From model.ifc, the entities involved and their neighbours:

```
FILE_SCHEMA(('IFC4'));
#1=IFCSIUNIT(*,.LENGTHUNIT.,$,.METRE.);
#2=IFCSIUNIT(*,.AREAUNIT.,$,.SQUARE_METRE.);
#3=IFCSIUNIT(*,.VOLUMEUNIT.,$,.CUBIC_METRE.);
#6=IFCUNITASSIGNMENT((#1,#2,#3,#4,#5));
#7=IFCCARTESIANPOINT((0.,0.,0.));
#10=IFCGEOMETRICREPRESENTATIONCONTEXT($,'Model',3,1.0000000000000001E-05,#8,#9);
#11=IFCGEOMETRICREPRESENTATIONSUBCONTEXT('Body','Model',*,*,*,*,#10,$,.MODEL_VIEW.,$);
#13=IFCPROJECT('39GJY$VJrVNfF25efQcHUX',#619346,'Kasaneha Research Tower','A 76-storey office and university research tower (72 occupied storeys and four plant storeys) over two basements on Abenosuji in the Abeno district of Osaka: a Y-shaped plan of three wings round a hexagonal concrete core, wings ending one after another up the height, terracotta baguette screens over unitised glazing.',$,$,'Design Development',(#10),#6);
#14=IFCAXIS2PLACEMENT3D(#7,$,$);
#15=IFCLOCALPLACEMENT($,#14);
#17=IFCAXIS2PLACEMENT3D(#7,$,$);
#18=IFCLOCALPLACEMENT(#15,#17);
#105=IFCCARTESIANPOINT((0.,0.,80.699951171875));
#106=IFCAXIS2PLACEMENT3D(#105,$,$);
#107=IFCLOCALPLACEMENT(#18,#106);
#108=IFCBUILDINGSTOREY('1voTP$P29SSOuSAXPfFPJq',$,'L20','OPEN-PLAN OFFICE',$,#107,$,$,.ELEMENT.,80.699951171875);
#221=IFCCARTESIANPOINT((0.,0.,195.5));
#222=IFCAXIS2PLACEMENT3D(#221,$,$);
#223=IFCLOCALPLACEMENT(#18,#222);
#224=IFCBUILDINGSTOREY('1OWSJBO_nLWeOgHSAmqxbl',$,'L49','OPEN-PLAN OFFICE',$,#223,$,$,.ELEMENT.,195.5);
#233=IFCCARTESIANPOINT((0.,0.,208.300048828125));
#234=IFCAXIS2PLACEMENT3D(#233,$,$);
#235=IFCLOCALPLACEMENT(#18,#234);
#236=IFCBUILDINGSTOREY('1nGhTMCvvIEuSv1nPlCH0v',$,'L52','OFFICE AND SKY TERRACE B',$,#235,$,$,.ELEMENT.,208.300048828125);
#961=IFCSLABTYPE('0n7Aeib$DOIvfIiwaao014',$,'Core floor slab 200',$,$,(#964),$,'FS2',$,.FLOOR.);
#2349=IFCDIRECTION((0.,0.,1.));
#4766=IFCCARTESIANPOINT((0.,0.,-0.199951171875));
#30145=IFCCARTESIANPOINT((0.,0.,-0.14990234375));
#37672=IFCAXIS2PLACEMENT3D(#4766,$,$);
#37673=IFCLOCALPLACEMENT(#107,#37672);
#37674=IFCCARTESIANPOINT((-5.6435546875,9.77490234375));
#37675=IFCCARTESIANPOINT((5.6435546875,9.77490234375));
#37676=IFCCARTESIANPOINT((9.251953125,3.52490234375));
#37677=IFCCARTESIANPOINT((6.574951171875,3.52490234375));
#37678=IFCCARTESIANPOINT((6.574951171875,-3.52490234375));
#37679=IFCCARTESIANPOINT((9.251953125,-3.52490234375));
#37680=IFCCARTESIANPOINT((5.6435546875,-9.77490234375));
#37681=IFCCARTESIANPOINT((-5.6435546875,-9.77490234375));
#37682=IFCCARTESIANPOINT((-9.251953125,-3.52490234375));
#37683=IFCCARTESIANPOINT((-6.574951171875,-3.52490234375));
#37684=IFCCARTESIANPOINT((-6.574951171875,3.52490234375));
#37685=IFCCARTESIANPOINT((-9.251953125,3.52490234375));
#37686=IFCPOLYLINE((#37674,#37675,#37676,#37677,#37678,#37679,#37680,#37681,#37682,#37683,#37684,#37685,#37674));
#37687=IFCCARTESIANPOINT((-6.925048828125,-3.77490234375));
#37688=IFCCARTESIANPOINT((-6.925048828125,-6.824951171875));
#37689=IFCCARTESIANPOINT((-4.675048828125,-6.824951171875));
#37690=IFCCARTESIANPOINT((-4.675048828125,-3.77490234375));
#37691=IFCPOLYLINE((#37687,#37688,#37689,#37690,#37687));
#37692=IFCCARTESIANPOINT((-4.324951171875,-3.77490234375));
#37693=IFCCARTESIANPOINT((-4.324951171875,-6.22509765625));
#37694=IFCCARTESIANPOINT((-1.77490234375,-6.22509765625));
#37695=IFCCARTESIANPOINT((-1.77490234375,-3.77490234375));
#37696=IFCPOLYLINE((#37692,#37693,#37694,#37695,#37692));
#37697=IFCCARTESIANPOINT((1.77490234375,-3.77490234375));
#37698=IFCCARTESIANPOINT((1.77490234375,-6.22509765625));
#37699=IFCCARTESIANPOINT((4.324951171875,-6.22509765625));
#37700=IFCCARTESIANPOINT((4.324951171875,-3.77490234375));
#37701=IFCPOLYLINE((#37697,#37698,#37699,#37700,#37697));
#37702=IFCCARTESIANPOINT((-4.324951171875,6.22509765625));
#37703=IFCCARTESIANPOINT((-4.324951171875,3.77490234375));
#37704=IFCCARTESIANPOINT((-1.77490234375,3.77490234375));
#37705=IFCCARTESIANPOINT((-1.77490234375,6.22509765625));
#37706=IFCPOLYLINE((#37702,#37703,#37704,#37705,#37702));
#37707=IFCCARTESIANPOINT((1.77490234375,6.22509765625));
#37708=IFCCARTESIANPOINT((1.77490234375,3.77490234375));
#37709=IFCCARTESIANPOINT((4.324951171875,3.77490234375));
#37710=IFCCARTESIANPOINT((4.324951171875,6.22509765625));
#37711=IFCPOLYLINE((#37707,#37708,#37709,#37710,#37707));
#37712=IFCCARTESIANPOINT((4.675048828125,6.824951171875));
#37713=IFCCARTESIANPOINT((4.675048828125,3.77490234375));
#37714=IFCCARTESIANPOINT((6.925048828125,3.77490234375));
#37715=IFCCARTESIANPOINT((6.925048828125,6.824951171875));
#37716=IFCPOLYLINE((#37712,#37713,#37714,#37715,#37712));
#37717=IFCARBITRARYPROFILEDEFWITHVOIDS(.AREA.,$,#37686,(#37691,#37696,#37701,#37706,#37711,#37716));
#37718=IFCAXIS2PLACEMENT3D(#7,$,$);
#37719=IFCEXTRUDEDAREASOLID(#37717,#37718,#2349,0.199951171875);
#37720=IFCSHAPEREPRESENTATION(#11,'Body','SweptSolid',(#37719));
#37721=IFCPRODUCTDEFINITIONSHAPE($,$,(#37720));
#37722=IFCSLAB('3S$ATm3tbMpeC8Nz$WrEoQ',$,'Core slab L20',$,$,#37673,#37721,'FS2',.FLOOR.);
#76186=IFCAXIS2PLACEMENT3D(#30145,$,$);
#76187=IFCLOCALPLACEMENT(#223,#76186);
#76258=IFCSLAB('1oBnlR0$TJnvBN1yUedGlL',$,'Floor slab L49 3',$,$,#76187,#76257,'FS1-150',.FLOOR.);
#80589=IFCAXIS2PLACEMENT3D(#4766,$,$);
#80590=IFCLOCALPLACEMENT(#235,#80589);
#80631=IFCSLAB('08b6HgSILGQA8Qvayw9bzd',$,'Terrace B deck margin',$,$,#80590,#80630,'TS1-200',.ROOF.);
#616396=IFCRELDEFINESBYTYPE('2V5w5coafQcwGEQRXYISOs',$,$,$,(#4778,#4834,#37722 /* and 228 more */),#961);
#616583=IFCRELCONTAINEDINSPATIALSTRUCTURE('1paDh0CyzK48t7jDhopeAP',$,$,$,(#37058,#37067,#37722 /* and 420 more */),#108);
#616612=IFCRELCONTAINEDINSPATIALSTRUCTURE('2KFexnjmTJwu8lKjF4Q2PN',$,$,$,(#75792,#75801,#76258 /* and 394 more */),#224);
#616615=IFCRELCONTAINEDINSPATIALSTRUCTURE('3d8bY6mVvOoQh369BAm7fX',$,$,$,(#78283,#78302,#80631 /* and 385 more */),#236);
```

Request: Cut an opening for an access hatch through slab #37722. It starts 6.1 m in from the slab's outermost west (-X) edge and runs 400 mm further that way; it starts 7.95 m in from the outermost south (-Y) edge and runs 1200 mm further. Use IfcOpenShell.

```python
import numpy as np
import ifcopenshell
import ifcopenshell.api.feature
import ifcopenshell.api.geometry
import ifcopenshell.api.root
import ifcopenshell.geom
import ifcopenshell.util.placement
import ifcopenshell.util.representation
import ifcopenshell.util.shape
import ifcopenshell.util.unit

model = ifcopenshell.open("model.ifc")
unit_scale = ifcopenshell.util.unit.calculate_unit_scale(model)
settings = ifcopenshell.geom.settings()


def volume(element):
    """Net volume in cubic metres, openings subtracted."""
    shape = ifcopenshell.geom.create_shape(settings, element)
    return ifcopenshell.util.shape.get_volume(shape.geometry)


slab = model.by_guid("3S$ATm3tbMpeC8Nz$WrEoQ")
before = volume(slab)

# Extent in the slab's own axes, in metres. The edges named are its -X and -Y sides.
slab_shape = ifcopenshell.geom.create_shape(settings, slab)
vertices = ifcopenshell.util.shape.get_vertices(slab_shape.geometry)
x_min, y_min, bottom = vertices.min(axis=0)
top = vertices[:, 2].max()

opening = ifcopenshell.api.root.create_entity(model, ifc_class="IfcOpeningElement", name="Access hatch opening", predefined_type="OPENING")
context = ifcopenshell.util.representation.get_context(model, "Model", "Body", "MODEL_VIEW")
width, depth = 0.4, 1.2
outline = [(0.0, 0.0), (width, 0.0), (width, depth), (0.0, depth), (0.0, 0.0)]
# Overshoot both faces by 50 mm so the cut is clean.
shape = ifcopenshell.api.geometry.add_slab_representation(
    model, context=context, depth=top - bottom + 0.1, polyline=outline
)
ifcopenshell.api.geometry.assign_representation(model, product=opening, representation=shape)

matrix = ifcopenshell.util.placement.get_local_placement(slab.ObjectPlacement)
matrix[:, 3] = matrix @ np.append(np.array([x_min + 6.1, y_min + 7.95, bottom - 0.05]) / unit_scale, 1.0)
ifcopenshell.api.geometry.edit_object_placement(model, product=opening, matrix=matrix, is_si=False)
ifcopenshell.api.feature.add_feature(model, feature=opening, element=slab)

after = volume(slab)

print(f"slab volume {before:.3f} -> {after:.3f} m3")

model.write("model_v2.ifc")
```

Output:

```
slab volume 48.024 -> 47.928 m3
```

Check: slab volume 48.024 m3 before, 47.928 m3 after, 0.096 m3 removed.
